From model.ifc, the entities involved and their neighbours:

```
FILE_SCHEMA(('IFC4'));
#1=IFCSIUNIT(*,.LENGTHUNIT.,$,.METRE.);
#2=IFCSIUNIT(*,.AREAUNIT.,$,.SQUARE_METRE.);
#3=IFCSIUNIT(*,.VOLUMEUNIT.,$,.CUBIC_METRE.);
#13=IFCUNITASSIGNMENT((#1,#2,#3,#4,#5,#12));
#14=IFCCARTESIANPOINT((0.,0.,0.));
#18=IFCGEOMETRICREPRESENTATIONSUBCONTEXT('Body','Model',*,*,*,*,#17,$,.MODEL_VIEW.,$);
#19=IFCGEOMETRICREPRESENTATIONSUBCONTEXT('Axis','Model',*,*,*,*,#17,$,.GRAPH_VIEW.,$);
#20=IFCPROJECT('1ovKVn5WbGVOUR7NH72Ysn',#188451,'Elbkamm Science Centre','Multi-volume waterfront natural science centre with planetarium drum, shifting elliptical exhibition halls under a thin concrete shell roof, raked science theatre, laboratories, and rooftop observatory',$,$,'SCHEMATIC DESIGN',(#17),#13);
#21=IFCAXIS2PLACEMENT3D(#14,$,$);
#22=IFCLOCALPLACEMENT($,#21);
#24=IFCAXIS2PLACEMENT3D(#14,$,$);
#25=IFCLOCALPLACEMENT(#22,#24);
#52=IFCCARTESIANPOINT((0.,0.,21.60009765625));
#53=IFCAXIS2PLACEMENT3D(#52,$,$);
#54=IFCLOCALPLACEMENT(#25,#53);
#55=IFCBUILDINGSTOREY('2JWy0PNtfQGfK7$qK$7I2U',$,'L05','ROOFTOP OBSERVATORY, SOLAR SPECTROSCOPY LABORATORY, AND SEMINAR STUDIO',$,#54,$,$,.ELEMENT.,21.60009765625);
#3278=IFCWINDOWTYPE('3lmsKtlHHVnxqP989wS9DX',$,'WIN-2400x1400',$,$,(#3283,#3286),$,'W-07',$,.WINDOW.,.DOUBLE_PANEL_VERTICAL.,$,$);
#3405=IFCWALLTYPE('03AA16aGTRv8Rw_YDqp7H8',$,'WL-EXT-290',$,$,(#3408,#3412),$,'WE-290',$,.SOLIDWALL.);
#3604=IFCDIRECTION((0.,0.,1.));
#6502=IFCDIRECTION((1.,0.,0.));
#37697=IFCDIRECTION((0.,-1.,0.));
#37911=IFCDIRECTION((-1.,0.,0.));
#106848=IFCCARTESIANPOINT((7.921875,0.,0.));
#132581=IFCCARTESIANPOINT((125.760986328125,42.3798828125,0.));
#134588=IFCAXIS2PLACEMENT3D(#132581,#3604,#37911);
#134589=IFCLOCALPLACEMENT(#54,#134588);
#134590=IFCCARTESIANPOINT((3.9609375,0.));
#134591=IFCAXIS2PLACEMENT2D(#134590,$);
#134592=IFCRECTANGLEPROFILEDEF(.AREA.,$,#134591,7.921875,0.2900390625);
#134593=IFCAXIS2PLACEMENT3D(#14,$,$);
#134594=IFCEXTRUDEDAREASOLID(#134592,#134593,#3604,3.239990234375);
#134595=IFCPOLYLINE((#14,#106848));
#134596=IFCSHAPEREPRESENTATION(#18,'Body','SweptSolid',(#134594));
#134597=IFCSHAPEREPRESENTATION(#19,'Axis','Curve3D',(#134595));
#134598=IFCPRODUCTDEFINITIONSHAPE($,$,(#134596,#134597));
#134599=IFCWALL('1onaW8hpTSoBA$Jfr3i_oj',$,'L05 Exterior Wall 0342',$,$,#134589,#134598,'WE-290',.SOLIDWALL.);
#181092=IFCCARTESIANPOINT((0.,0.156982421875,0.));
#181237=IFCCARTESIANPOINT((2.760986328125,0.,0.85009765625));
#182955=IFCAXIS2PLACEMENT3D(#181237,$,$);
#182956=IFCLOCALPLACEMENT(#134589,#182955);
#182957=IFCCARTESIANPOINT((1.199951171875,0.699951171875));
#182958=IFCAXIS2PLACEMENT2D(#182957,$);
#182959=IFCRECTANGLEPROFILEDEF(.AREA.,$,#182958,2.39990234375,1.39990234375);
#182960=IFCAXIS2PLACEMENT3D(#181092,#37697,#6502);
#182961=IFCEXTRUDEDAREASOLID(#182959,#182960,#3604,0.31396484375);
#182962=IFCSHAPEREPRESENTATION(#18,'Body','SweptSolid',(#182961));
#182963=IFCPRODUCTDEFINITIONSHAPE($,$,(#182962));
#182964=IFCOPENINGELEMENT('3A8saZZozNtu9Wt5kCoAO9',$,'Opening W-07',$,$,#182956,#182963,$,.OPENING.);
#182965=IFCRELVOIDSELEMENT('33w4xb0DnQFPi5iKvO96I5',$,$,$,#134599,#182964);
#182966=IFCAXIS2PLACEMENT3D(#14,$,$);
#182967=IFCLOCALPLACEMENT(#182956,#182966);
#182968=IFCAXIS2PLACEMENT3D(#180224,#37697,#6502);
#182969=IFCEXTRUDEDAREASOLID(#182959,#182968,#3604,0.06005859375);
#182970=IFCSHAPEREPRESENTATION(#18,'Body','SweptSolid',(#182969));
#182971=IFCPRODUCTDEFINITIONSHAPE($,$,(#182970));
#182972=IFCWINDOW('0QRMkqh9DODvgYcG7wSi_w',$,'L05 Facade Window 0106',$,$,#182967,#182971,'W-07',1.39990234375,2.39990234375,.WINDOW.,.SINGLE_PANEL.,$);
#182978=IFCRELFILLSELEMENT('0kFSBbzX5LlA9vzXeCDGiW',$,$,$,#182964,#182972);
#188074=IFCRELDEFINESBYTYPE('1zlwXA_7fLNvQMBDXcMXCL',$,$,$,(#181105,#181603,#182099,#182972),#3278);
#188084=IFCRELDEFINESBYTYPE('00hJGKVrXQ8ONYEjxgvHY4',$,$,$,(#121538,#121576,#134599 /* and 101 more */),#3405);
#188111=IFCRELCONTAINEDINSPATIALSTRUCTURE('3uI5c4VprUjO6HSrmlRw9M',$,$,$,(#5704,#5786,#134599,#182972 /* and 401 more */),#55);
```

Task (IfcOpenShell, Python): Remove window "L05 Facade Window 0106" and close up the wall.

```python
import ifcopenshell
import ifcopenshell.api.feature
import ifcopenshell.api.root
import ifcopenshell.geom
import ifcopenshell.util.shape

model = ifcopenshell.open("model.ifc")
settings = ifcopenshell.geom.settings()


def volume(element):
    """Net volume in cubic metres, openings subtracted."""
    shape = ifcopenshell.geom.create_shape(settings, element)
    return ifcopenshell.util.shape.get_volume(shape.geometry)


window = model.by_guid("0QRMkqh9DODvgYcG7wSi_w")
opening = window.FillsVoids[0].RelatingOpeningElement
wall = opening.VoidsElements[0].RelatingBuildingElement
before = volume(wall)

ifcopenshell.api.root.remove_product(model, product=window)
ifcopenshell.api.feature.remove_feature(model, feature=opening)

after = volume(wall)

print(f"wall volume {before:.3f} -> {after:.3f} m3")

model.write("model-out.ifc")
```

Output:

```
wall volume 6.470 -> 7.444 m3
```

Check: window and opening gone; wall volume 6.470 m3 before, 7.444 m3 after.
